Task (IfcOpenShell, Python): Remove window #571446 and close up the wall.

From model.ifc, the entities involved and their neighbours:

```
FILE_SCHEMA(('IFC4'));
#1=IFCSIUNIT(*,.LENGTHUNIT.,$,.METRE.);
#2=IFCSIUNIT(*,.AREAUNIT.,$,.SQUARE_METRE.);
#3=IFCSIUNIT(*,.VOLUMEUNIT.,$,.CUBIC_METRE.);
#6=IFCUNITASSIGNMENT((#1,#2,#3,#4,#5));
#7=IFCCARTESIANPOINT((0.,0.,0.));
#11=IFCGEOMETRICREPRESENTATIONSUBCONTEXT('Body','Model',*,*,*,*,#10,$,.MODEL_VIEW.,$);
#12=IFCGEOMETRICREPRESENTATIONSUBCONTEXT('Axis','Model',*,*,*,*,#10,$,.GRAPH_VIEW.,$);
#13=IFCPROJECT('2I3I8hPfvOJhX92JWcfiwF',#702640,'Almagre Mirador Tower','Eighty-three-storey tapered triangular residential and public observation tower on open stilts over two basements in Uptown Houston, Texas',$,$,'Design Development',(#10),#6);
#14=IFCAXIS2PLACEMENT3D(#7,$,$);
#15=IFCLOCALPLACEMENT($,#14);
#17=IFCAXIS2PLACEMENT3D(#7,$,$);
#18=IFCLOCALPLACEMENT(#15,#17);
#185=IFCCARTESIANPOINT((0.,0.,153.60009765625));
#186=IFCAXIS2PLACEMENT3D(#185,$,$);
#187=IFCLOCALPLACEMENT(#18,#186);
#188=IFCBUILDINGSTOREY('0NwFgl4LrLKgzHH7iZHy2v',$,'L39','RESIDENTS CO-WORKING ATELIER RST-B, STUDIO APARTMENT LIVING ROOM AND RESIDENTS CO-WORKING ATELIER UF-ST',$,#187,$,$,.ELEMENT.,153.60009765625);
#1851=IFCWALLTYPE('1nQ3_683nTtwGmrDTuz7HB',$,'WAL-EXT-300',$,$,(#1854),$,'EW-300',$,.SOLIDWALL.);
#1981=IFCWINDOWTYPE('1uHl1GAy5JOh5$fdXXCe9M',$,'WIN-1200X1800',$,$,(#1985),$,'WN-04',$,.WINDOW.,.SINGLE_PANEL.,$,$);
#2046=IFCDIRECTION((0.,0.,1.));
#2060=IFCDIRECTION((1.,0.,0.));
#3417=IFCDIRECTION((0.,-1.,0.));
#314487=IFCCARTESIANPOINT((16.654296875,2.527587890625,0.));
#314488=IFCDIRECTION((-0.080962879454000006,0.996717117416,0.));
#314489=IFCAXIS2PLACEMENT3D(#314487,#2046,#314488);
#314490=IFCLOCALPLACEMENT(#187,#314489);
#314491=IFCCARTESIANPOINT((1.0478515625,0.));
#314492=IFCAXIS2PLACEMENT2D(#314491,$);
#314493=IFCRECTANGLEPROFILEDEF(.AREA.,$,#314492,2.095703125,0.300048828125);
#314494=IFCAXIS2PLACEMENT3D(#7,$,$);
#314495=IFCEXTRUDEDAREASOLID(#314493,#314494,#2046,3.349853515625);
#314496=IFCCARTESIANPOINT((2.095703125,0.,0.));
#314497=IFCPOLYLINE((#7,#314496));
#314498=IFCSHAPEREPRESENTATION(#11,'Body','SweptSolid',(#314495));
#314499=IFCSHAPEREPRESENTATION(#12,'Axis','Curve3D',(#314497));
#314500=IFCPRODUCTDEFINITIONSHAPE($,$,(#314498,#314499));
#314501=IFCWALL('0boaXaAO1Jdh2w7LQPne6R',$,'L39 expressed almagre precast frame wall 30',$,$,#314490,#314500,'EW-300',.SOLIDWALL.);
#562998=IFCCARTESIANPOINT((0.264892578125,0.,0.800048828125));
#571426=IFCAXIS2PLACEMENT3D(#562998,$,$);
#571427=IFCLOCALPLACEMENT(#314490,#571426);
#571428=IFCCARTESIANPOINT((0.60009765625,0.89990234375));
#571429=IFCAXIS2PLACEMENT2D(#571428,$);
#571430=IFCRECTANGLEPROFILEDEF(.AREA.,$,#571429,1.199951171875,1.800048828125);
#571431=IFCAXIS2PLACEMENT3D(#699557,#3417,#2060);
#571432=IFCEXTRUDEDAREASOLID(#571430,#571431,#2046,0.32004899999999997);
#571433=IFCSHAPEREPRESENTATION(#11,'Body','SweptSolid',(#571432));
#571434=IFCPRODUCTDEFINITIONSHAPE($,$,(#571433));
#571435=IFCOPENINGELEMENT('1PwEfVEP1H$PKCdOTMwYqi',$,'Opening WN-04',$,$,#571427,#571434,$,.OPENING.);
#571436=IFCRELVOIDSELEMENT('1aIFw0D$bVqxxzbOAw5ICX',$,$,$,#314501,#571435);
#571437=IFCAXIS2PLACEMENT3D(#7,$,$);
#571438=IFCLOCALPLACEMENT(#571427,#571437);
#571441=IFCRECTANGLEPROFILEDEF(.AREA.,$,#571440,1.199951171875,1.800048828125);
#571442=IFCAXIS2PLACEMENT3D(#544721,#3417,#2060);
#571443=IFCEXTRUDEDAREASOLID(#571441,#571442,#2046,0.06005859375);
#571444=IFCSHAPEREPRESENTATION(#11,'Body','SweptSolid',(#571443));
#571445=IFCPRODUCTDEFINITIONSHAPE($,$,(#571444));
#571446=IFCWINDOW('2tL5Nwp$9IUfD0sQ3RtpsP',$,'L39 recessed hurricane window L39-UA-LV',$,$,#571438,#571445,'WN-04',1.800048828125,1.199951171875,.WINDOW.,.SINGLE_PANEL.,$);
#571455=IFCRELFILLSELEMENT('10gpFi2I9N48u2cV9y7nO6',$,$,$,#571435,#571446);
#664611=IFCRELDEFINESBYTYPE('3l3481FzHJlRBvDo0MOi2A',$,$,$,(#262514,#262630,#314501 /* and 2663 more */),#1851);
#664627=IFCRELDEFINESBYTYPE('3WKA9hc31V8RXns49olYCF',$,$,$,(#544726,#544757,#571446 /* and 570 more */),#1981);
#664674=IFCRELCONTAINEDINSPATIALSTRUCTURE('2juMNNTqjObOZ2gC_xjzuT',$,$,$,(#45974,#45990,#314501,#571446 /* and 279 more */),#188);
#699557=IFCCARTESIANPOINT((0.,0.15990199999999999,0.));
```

```python
import ifcopenshell
import ifcopenshell.api.feature
import ifcopenshell.api.root
import ifcopenshell.geom
import ifcopenshell.util.shape

model = ifcopenshell.open("model.ifc")
settings = ifcopenshell.geom.settings()


def volume(element):
    """Net volume in cubic metres, openings subtracted."""
    shape = ifcopenshell.geom.create_shape(settings, element)
    return ifcopenshell.util.shape.get_volume(shape.geometry)


window = model.by_guid("2tL5Nwp$9IUfD0sQ3RtpsP")
opening = window.FillsVoids[0].RelatingOpeningElement
wall = opening.VoidsElements[0].RelatingBuildingElement
before = volume(wall)

ifcopenshell.api.root.remove_product(model, product=window)
ifcopenshell.api.feature.remove_feature(model, feature=opening)

after = volume(wall)

print(f"wall volume {before:.3f} -> {after:.3f} m3")

model.write("model_rev.ifc")
```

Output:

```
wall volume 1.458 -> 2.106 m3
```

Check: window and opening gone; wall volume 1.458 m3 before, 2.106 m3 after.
